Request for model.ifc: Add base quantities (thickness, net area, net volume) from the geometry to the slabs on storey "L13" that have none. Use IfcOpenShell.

First a look at what the model holds.

```python
import ifcopenshell
import ifcopenshell.util.element
import ifcopenshell.util.unit

model = ifcopenshell.open("model.ifc")
print(model.schema)
for unit_type in ("LENGTHUNIT", "AREAUNIT", "VOLUMEUNIT"):
    print(unit_type, ifcopenshell.util.unit.calculate_unit_scale(model, unit_type))
storey = next(s for s in model.by_type("IfcBuildingStorey") if s.Name == "L13")
slabs = [e for e in ifcopenshell.util.element.get_decomposition(storey) if e.is_a("IfcSlab")]
for e in sorted(slabs, key=lambda e: e.id()):
    print(e.id(), e.is_a(), e.Name, list(ifcopenshell.util.element.get_psets(e, qtos_only=True)), sep=" | ")
```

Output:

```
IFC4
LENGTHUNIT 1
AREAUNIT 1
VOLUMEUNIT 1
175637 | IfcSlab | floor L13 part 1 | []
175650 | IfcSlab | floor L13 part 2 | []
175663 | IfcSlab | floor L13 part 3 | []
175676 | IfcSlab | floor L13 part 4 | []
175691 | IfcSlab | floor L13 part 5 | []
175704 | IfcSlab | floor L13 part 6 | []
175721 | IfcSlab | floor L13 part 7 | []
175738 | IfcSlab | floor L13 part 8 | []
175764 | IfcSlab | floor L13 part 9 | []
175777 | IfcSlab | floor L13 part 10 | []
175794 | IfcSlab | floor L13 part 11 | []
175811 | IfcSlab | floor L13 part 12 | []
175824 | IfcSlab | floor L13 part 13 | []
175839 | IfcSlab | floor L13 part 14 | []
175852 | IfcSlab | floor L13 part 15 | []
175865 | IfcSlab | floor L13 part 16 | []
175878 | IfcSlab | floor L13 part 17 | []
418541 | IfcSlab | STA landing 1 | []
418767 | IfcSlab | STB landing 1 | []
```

```python
import ifcopenshell
import ifcopenshell.api.pset
import ifcopenshell.geom
import ifcopenshell.util.element
import ifcopenshell.util.shape
import ifcopenshell.util.unit

model = ifcopenshell.open("model.ifc")
unit_scale = ifcopenshell.util.unit.calculate_unit_scale(model)
area_scale = ifcopenshell.util.unit.calculate_unit_scale(model, "AREAUNIT")
volume_scale = ifcopenshell.util.unit.calculate_unit_scale(model, "VOLUMEUNIT")
settings = ifcopenshell.geom.settings()

storey = next(s for s in model.by_type("IfcBuildingStorey") if s.Name == "L13")
slabs = [e for e in ifcopenshell.util.element.get_decomposition(storey) if e.is_a("IfcSlab")]

for e in sorted(slabs, key=lambda e: e.id()):
    if ifcopenshell.util.element.get_psets(e, qtos_only=True, should_inherit=False):
        continue
    # Geometry comes back in metres, in the element's own axes.
    shape = ifcopenshell.geom.create_shape(settings, e)
    values = {
        "Width": ifcopenshell.util.shape.get_z(shape.geometry) / unit_scale,
        "NetArea": ifcopenshell.util.shape.get_footprint_area(shape.geometry) / area_scale,
        "NetVolume": ifcopenshell.util.shape.get_volume(shape.geometry) / volume_scale,
    }
    qto = ifcopenshell.api.pset.add_qto(model, product=e, name="Qto_SlabBaseQuantities")
    ifcopenshell.api.pset.edit_qto(model, qto=qto, properties=values)
    print(e.id(), {k: round(v, 3) for k, v in values.items()})

model.write("model_edited.ifc")
```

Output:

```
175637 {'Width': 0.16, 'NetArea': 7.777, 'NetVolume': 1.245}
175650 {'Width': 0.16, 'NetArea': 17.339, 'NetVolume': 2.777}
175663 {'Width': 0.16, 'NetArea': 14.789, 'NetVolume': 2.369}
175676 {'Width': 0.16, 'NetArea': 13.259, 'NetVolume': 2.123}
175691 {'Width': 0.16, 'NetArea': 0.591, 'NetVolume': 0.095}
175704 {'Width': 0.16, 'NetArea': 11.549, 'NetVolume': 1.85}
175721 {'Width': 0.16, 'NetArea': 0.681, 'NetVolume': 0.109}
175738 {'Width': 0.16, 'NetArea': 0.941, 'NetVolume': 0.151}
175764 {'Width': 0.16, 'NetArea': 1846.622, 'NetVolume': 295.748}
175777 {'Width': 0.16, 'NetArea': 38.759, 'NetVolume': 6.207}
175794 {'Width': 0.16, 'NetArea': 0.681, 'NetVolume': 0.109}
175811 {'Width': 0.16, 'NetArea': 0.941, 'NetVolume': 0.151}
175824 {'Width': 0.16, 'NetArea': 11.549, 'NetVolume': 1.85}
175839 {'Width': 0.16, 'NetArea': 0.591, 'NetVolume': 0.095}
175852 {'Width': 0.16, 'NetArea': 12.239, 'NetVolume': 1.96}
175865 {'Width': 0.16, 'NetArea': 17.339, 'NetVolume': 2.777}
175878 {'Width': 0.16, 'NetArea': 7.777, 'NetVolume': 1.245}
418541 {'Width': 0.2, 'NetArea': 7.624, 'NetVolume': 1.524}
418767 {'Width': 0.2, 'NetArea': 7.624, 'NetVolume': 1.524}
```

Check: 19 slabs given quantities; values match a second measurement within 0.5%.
